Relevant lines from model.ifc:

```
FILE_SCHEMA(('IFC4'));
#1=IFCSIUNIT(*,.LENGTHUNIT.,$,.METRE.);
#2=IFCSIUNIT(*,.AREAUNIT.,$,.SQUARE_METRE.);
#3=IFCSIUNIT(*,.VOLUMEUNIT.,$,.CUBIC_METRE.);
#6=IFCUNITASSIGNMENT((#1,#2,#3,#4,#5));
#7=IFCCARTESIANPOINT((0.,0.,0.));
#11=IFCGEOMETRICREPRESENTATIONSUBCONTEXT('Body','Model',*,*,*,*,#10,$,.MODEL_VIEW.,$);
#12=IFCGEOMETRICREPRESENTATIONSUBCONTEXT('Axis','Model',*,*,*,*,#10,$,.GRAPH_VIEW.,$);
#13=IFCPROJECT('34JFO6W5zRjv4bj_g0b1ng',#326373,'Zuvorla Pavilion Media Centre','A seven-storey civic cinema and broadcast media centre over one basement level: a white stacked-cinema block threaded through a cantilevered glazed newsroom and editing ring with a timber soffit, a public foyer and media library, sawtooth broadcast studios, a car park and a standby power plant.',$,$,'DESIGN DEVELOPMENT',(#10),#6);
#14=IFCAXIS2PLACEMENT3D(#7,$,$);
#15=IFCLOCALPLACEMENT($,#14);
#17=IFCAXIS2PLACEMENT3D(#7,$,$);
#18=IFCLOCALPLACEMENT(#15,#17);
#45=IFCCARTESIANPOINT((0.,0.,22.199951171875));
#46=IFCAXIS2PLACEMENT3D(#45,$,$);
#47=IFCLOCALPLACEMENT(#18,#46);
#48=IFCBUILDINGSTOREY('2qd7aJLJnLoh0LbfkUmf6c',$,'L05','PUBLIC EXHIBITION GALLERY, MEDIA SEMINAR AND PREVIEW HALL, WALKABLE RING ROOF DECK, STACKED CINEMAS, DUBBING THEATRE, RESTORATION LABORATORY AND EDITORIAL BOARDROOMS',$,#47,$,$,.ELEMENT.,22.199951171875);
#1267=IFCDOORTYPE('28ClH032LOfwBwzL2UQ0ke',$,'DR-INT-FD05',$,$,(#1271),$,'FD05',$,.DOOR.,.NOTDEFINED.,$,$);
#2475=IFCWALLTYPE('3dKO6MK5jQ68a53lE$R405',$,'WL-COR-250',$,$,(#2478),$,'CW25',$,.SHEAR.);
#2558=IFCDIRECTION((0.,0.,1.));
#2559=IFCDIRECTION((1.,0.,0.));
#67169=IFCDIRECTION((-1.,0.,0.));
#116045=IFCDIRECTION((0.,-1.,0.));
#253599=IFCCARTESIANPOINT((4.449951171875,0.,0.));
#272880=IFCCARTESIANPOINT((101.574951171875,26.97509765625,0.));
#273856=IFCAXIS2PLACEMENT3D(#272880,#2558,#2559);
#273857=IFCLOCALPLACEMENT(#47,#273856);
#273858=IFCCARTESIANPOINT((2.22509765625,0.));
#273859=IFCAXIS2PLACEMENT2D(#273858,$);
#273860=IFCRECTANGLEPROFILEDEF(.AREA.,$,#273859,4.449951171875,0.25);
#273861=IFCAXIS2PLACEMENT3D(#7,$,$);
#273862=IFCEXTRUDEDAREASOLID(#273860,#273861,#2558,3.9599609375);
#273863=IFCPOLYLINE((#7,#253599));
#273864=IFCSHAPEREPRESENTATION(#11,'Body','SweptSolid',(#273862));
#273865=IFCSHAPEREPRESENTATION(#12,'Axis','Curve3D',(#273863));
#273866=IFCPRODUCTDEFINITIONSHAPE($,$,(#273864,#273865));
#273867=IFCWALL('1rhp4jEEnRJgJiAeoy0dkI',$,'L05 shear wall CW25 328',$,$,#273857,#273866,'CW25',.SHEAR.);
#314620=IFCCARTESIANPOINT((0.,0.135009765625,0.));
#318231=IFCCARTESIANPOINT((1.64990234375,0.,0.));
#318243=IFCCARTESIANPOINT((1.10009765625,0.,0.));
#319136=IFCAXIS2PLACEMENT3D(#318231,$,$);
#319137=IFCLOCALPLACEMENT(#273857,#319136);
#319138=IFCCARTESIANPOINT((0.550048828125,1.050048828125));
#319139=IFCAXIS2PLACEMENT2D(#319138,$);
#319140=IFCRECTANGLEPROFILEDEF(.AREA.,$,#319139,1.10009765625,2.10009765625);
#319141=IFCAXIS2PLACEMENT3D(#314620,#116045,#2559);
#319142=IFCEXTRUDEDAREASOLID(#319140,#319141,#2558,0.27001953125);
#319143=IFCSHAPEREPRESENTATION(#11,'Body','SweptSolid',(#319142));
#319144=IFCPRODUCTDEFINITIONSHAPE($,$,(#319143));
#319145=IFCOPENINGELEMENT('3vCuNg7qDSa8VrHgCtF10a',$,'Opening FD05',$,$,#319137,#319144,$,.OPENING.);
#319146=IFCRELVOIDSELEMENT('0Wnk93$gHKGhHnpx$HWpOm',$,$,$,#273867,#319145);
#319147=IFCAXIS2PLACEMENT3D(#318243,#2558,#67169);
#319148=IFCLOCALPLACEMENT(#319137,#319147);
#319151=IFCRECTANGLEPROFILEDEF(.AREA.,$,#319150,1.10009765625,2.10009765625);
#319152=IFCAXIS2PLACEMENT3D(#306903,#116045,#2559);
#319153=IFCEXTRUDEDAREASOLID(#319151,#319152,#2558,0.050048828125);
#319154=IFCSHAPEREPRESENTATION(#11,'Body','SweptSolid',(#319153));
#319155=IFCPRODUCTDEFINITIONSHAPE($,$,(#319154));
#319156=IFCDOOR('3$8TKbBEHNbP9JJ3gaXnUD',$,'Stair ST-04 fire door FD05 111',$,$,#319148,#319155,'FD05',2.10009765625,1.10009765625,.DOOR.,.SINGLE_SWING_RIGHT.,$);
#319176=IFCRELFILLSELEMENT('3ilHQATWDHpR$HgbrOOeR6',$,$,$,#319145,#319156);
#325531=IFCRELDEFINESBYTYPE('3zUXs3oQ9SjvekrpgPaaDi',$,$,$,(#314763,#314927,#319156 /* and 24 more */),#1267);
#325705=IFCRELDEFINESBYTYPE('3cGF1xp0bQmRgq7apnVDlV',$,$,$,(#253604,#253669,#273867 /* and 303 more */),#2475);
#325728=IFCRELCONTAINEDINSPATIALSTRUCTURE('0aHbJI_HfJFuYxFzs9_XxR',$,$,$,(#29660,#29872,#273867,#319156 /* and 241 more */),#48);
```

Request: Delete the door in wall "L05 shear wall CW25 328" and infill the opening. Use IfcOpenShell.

```python
import ifcopenshell
import ifcopenshell.api.feature
import ifcopenshell.api.root
import ifcopenshell.geom
import ifcopenshell.util.shape

model = ifcopenshell.open("model.ifc")
settings = ifcopenshell.geom.settings()


def volume(element):
    """Net volume in cubic metres, openings subtracted."""
    shape = ifcopenshell.geom.create_shape(settings, element)
    return ifcopenshell.util.shape.get_volume(shape.geometry)


door = model.by_guid("3$8TKbBEHNbP9JJ3gaXnUD")
opening = door.FillsVoids[0].RelatingOpeningElement
wall = opening.VoidsElements[0].RelatingBuildingElement
before = volume(wall)

ifcopenshell.api.root.remove_product(model, product=door)
ifcopenshell.api.feature.remove_feature(model, feature=opening)

after = volume(wall)

print(f"wall volume {before:.3f} -> {after:.3f} m3")

model.write("model_updated.ifc")
```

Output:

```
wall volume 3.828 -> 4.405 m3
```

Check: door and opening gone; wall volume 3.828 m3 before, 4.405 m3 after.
